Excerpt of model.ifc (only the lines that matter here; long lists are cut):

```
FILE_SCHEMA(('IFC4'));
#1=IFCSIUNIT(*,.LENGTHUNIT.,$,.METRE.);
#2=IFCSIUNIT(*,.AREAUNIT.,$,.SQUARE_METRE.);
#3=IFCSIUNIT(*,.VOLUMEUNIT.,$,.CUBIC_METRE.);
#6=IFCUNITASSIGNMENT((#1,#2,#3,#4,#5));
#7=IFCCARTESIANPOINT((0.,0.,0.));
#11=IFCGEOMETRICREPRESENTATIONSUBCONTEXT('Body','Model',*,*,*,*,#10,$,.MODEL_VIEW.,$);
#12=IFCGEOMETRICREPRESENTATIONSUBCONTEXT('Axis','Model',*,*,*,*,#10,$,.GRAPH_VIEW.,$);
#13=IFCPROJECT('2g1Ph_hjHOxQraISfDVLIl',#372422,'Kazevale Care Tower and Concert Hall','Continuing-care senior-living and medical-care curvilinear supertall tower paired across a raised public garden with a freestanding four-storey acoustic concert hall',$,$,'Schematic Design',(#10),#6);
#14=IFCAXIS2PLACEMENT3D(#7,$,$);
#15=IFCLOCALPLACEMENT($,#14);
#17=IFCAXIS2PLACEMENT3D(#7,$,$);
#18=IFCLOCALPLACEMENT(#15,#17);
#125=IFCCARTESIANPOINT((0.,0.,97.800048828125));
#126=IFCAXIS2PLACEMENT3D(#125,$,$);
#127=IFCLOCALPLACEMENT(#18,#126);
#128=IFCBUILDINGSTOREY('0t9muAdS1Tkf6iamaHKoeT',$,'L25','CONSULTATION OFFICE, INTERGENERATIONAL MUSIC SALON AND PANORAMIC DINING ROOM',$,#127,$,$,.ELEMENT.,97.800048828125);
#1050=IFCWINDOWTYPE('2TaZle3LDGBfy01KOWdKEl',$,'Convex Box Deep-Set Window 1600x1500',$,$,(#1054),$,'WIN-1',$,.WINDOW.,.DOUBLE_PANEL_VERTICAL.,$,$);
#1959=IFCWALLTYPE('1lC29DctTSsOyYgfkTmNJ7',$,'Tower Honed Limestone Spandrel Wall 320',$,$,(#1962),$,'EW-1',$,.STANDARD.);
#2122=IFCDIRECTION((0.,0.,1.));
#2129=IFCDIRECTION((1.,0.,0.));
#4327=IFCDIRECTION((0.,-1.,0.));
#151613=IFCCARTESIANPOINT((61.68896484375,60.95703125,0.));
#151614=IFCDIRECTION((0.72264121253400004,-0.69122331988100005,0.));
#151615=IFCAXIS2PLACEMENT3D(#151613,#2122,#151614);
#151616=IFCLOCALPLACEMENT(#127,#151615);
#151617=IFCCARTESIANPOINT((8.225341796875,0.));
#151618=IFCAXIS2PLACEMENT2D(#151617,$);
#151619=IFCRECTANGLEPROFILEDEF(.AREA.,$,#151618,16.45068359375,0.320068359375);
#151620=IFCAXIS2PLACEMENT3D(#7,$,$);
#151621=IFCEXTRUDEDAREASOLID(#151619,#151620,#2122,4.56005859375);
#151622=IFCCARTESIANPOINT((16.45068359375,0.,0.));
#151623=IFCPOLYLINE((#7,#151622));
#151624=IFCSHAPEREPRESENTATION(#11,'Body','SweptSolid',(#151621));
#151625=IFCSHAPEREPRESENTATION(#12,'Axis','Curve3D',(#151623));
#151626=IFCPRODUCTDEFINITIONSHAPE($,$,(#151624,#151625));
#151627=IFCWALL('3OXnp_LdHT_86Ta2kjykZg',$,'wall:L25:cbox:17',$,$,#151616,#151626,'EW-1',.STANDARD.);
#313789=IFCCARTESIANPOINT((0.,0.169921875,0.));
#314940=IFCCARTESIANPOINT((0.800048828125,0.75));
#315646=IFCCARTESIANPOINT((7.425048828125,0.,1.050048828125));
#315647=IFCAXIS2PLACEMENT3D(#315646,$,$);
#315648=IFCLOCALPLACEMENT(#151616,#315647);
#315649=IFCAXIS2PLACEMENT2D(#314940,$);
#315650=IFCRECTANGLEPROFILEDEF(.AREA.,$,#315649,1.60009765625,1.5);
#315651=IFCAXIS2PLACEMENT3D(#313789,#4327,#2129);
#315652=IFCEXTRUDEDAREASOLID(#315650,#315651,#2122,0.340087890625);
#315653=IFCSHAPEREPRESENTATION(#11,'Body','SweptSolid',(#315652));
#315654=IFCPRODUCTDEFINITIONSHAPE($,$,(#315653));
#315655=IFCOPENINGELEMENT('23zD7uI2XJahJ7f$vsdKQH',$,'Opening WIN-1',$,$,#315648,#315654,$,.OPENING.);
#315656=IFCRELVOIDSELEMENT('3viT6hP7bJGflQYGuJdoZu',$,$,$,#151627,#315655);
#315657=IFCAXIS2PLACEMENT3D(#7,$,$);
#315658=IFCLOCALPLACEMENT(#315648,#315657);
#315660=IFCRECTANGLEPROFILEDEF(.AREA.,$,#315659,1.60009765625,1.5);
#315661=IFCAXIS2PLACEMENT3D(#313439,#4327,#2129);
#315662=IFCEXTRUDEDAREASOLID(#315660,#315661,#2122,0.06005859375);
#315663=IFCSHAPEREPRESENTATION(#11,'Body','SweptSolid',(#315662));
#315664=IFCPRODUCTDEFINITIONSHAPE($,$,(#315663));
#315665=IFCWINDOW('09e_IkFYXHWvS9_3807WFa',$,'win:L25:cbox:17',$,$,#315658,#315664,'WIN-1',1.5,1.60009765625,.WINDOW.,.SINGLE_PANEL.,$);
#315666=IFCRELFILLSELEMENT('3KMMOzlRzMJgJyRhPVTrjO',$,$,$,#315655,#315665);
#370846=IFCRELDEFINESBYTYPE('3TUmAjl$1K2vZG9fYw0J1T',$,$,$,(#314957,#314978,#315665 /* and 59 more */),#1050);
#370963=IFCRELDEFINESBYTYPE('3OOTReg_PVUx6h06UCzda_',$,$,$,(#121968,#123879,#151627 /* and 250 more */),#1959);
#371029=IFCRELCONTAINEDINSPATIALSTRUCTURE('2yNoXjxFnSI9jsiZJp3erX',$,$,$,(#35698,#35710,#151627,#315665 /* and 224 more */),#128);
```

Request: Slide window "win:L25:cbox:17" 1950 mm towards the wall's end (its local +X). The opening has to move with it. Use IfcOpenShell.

```python
import ifcopenshell
import ifcopenshell.api.geometry
import ifcopenshell.util.placement
import ifcopenshell.util.unit

model = ifcopenshell.open("model.ifc")
unit_scale = ifcopenshell.util.unit.calculate_unit_scale(model)

window = model.by_id(315665)
opening = window.FillsVoids[0].RelatingOpeningElement
wall = opening.VoidsElements[0].RelatingBuildingElement

wall_matrix = ifcopenshell.util.placement.get_local_placement(wall.ObjectPlacement)
shift = wall_matrix[:3, 0] * 1.95 / unit_scale
before = ifcopenshell.util.placement.get_local_placement(window.ObjectPlacement)[:3, 3].copy()

# The window is placed relative to its opening, so it follows when the opening moves.
matrix = ifcopenshell.util.placement.get_local_placement(opening.ObjectPlacement)
matrix[:3, 3] += shift
ifcopenshell.api.geometry.edit_object_placement(
    model, product=opening, matrix=matrix, is_si=False, should_transform_children=True
)

after = ifcopenshell.util.placement.get_local_placement(window.ObjectPlacement)[:3, 3]
print("window moved by", (after - before).round(3) + 0.0)

model.write("model_rev.ifc")
```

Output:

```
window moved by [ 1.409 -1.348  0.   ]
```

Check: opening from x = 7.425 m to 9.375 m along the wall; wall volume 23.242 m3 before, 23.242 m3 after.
